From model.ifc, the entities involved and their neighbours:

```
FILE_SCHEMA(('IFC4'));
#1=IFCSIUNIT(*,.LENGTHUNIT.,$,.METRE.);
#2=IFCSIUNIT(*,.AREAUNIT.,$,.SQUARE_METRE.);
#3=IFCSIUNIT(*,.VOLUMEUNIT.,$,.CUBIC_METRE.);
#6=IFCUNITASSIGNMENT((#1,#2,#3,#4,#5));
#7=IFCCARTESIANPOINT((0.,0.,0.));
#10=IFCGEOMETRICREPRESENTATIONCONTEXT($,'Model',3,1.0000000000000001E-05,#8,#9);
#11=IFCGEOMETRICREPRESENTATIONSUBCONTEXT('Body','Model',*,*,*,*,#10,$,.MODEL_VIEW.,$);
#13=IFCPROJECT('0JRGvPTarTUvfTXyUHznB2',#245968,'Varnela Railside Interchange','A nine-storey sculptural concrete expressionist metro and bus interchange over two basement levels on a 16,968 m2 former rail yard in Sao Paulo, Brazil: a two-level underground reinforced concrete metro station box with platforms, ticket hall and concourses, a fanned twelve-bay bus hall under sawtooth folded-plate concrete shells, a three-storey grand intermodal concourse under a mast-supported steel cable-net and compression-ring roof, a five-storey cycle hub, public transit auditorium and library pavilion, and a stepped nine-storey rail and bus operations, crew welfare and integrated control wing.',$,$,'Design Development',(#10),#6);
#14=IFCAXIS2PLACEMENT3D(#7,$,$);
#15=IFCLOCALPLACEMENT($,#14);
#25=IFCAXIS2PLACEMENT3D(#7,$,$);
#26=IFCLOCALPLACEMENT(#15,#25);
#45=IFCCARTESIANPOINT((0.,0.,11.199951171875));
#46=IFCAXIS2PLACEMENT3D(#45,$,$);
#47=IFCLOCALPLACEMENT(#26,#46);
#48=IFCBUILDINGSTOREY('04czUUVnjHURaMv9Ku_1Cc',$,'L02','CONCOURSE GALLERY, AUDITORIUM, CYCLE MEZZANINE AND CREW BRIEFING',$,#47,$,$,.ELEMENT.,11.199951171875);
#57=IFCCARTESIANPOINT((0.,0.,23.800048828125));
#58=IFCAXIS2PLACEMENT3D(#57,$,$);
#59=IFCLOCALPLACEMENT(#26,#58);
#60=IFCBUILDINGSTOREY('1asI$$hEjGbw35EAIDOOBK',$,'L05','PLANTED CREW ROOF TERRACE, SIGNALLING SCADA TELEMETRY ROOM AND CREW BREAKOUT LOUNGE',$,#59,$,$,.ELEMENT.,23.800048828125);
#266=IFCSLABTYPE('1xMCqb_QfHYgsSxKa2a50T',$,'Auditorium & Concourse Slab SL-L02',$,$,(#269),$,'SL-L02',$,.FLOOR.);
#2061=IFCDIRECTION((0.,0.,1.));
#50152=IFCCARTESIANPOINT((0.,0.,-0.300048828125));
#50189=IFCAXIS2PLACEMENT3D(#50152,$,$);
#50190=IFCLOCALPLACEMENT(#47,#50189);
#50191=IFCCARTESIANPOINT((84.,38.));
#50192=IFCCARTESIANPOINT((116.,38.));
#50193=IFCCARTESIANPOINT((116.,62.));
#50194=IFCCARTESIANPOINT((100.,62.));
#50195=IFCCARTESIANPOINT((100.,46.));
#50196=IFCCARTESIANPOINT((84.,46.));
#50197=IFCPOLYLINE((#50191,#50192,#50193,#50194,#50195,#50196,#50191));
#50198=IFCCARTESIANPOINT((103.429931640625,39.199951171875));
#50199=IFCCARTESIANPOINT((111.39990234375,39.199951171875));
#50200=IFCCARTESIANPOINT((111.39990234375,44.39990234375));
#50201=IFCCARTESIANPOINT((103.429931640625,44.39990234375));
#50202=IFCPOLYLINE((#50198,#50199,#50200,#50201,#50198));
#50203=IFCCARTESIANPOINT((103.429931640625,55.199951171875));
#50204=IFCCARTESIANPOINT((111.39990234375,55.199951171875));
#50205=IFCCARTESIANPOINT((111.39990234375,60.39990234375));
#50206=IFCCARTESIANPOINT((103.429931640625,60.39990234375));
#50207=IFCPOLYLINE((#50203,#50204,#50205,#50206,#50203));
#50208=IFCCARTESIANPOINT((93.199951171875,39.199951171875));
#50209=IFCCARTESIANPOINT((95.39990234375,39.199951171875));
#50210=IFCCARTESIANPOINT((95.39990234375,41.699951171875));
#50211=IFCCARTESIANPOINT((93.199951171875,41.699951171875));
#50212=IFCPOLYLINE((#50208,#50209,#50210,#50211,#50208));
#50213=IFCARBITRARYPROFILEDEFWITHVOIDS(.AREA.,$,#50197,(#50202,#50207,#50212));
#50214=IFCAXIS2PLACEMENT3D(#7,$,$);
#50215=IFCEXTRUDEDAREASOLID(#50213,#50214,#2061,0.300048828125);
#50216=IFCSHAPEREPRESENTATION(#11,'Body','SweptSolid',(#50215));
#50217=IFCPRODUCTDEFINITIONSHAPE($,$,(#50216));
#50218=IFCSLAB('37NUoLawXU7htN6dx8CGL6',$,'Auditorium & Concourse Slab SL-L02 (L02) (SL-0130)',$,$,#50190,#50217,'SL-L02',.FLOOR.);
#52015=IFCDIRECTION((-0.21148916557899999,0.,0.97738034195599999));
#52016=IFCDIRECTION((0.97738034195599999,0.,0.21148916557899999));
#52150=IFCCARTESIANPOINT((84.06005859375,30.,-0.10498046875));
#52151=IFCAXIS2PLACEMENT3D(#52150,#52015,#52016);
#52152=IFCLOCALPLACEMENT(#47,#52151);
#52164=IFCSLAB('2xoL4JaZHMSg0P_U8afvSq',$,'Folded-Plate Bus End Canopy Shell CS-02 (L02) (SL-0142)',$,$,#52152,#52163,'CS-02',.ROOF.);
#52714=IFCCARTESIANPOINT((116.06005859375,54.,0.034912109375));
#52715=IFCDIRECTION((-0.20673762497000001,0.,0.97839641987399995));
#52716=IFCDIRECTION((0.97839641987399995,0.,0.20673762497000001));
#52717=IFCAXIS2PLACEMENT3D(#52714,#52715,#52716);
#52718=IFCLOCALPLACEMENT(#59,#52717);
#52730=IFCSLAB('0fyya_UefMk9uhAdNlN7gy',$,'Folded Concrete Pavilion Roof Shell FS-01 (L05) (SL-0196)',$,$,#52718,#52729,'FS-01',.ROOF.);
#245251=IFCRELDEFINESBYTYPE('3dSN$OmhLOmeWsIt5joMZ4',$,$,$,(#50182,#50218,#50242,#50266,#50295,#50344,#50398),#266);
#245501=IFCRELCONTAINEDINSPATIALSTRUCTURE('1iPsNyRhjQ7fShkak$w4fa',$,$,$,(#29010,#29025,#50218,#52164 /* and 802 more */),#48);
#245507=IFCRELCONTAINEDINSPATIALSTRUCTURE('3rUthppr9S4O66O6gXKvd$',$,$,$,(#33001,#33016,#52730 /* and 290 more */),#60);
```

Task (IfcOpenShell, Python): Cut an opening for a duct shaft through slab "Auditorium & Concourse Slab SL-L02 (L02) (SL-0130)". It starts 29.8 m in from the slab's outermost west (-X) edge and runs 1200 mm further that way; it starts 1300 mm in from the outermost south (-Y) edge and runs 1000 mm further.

```python
import numpy as np
import ifcopenshell
import ifcopenshell.api.feature
import ifcopenshell.api.geometry
import ifcopenshell.api.root
import ifcopenshell.geom
import ifcopenshell.util.placement
import ifcopenshell.util.representation
import ifcopenshell.util.shape
import ifcopenshell.util.unit

model = ifcopenshell.open("model.ifc")
unit_scale = ifcopenshell.util.unit.calculate_unit_scale(model)
settings = ifcopenshell.geom.settings()


def volume(element):
    """Net volume in cubic metres, openings subtracted."""
    shape = ifcopenshell.geom.create_shape(settings, element)
    return ifcopenshell.util.shape.get_volume(shape.geometry)


slab = model.by_guid("37NUoLawXU7htN6dx8CGL6")
before = volume(slab)

# Extent in the slab's own axes, in metres. The edges named are its -X and -Y sides.
slab_shape = ifcopenshell.geom.create_shape(settings, slab)
vertices = ifcopenshell.util.shape.get_vertices(slab_shape.geometry)
x_min, y_min, bottom = vertices.min(axis=0)
top = vertices[:, 2].max()

opening = ifcopenshell.api.root.create_entity(model, ifc_class="IfcOpeningElement", name="Duct shaft opening", predefined_type="OPENING")
context = ifcopenshell.util.representation.get_context(model, "Model", "Body", "MODEL_VIEW")
width, depth = 1.2, 1
outline = [(0.0, 0.0), (width, 0.0), (width, depth), (0.0, depth), (0.0, 0.0)]
# Overshoot both faces by 50 mm so the cut is clean.
shape = ifcopenshell.api.geometry.add_slab_representation(
    model, context=context, depth=top - bottom + 0.1, polyline=outline
)
ifcopenshell.api.geometry.assign_representation(model, product=opening, representation=shape)

matrix = ifcopenshell.util.placement.get_local_placement(slab.ObjectPlacement)
matrix[:, 3] = matrix @ np.append(np.array([x_min + 29.8, y_min + 1.3, bottom - 0.05]) / unit_scale, 1.0)
ifcopenshell.api.geometry.edit_object_placement(model, product=opening, matrix=matrix, is_si=False)
ifcopenshell.api.feature.add_feature(model, feature=opening, element=slab)

after = volume(slab)

print(f"slab volume {before:.3f} -> {after:.3f} m3")

model.write("model_updated.ifc")
```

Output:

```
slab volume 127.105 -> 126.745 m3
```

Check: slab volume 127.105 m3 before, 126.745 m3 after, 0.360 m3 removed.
